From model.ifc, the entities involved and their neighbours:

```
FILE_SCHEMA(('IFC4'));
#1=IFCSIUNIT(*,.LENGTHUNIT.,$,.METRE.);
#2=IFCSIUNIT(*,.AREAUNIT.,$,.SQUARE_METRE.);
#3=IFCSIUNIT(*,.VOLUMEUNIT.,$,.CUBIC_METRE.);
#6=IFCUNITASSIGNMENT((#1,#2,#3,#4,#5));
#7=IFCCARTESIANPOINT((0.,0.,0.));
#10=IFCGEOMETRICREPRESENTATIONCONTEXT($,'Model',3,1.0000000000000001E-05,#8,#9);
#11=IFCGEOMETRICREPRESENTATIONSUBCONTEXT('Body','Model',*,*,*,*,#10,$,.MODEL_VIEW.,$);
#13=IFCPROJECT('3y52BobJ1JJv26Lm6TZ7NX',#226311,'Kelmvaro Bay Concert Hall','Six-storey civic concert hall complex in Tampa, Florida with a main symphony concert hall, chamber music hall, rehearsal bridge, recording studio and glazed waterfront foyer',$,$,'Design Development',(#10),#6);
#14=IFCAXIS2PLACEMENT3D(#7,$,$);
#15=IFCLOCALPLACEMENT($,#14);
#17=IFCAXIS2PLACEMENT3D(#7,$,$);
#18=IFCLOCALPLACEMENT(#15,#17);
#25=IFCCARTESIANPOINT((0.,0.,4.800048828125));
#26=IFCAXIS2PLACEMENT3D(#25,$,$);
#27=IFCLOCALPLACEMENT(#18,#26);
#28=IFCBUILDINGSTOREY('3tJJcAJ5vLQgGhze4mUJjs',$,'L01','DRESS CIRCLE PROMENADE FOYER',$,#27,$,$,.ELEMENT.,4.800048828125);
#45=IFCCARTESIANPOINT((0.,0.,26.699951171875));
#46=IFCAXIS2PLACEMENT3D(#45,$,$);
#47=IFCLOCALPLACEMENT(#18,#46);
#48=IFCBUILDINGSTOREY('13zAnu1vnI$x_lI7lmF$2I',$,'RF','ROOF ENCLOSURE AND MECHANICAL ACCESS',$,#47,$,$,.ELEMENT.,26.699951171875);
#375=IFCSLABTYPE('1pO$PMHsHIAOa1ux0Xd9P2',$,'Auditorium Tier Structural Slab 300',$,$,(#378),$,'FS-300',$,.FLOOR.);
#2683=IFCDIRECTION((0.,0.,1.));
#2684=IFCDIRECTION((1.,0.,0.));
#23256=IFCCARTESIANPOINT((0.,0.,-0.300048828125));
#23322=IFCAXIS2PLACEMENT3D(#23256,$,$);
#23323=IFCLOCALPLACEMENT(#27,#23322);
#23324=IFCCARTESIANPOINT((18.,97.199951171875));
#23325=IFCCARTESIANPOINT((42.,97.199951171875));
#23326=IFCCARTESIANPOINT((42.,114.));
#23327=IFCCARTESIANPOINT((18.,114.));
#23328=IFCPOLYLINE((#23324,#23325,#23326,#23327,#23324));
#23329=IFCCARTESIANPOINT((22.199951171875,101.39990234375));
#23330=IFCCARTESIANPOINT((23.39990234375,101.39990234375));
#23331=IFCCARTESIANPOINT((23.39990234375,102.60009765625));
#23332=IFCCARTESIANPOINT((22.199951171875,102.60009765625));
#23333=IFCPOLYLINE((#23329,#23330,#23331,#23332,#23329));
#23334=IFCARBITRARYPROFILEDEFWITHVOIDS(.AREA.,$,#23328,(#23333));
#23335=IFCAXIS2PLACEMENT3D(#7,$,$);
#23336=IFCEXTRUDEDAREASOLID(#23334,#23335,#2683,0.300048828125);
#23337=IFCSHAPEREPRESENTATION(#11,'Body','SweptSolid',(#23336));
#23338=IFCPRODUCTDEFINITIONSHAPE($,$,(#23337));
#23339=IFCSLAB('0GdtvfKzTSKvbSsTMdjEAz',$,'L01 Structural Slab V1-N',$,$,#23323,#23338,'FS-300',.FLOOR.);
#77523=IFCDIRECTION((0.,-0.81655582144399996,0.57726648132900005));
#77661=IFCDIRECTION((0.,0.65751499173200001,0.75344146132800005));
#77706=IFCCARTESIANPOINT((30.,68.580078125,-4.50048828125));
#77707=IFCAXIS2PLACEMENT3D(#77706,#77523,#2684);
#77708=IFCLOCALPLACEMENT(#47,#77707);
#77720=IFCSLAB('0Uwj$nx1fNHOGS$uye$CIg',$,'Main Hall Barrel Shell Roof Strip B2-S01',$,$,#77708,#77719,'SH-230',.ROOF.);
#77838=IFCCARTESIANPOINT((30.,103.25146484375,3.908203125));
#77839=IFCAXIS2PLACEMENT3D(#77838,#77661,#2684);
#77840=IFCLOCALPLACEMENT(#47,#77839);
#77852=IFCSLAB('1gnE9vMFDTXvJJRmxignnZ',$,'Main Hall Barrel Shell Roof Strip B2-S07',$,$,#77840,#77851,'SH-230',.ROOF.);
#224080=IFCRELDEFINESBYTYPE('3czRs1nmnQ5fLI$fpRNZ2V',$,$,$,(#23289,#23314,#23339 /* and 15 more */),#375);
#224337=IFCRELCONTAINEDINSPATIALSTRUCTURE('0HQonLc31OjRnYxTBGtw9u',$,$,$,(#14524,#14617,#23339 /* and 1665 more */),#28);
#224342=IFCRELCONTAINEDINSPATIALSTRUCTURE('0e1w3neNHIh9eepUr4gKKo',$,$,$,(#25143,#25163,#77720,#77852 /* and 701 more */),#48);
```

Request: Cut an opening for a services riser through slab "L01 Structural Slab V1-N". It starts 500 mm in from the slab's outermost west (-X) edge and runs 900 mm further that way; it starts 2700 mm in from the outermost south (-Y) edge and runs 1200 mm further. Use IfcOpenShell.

```python
import numpy as np
import ifcopenshell
import ifcopenshell.api.feature
import ifcopenshell.api.geometry
import ifcopenshell.api.root
import ifcopenshell.geom
import ifcopenshell.util.placement
import ifcopenshell.util.representation
import ifcopenshell.util.shape
import ifcopenshell.util.unit

model = ifcopenshell.open("model.ifc")
unit_scale = ifcopenshell.util.unit.calculate_unit_scale(model)
settings = ifcopenshell.geom.settings()


def volume(element):
    """Net volume in cubic metres, openings subtracted."""
    shape = ifcopenshell.geom.create_shape(settings, element)
    return ifcopenshell.util.shape.get_volume(shape.geometry)


slab = model.by_guid("0GdtvfKzTSKvbSsTMdjEAz")
before = volume(slab)

# Extent in the slab's own axes, in metres. The edges named are its -X and -Y sides.
slab_shape = ifcopenshell.geom.create_shape(settings, slab)
vertices = ifcopenshell.util.shape.get_vertices(slab_shape.geometry)
x_min, y_min, bottom = vertices.min(axis=0)
top = vertices[:, 2].max()

opening = ifcopenshell.api.root.create_entity(model, ifc_class="IfcOpeningElement", name="Services riser opening", predefined_type="OPENING")
context = ifcopenshell.util.representation.get_context(model, "Model", "Body", "MODEL_VIEW")
width, depth = 0.9, 1.2
outline = [(0.0, 0.0), (width, 0.0), (width, depth), (0.0, depth), (0.0, 0.0)]
# Overshoot both faces by 50 mm so the cut is clean.
shape = ifcopenshell.api.geometry.add_slab_representation(
    model, context=context, depth=top - bottom + 0.1, polyline=outline
)
ifcopenshell.api.geometry.assign_representation(model, product=opening, representation=shape)

matrix = ifcopenshell.util.placement.get_local_placement(slab.ObjectPlacement)
matrix[:, 3] = matrix @ np.append(np.array([x_min + 0.5, y_min + 2.7, bottom - 0.05]) / unit_scale, 1.0)
ifcopenshell.api.geometry.edit_object_placement(model, product=opening, matrix=matrix, is_si=False)
ifcopenshell.api.feature.add_feature(model, feature=opening, element=slab)

after = volume(slab)

print(f"slab volume {before:.3f} -> {after:.3f} m3")

model.write("model_v2.ifc")
```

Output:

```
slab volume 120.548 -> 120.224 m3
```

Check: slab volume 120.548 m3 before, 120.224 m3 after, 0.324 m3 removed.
